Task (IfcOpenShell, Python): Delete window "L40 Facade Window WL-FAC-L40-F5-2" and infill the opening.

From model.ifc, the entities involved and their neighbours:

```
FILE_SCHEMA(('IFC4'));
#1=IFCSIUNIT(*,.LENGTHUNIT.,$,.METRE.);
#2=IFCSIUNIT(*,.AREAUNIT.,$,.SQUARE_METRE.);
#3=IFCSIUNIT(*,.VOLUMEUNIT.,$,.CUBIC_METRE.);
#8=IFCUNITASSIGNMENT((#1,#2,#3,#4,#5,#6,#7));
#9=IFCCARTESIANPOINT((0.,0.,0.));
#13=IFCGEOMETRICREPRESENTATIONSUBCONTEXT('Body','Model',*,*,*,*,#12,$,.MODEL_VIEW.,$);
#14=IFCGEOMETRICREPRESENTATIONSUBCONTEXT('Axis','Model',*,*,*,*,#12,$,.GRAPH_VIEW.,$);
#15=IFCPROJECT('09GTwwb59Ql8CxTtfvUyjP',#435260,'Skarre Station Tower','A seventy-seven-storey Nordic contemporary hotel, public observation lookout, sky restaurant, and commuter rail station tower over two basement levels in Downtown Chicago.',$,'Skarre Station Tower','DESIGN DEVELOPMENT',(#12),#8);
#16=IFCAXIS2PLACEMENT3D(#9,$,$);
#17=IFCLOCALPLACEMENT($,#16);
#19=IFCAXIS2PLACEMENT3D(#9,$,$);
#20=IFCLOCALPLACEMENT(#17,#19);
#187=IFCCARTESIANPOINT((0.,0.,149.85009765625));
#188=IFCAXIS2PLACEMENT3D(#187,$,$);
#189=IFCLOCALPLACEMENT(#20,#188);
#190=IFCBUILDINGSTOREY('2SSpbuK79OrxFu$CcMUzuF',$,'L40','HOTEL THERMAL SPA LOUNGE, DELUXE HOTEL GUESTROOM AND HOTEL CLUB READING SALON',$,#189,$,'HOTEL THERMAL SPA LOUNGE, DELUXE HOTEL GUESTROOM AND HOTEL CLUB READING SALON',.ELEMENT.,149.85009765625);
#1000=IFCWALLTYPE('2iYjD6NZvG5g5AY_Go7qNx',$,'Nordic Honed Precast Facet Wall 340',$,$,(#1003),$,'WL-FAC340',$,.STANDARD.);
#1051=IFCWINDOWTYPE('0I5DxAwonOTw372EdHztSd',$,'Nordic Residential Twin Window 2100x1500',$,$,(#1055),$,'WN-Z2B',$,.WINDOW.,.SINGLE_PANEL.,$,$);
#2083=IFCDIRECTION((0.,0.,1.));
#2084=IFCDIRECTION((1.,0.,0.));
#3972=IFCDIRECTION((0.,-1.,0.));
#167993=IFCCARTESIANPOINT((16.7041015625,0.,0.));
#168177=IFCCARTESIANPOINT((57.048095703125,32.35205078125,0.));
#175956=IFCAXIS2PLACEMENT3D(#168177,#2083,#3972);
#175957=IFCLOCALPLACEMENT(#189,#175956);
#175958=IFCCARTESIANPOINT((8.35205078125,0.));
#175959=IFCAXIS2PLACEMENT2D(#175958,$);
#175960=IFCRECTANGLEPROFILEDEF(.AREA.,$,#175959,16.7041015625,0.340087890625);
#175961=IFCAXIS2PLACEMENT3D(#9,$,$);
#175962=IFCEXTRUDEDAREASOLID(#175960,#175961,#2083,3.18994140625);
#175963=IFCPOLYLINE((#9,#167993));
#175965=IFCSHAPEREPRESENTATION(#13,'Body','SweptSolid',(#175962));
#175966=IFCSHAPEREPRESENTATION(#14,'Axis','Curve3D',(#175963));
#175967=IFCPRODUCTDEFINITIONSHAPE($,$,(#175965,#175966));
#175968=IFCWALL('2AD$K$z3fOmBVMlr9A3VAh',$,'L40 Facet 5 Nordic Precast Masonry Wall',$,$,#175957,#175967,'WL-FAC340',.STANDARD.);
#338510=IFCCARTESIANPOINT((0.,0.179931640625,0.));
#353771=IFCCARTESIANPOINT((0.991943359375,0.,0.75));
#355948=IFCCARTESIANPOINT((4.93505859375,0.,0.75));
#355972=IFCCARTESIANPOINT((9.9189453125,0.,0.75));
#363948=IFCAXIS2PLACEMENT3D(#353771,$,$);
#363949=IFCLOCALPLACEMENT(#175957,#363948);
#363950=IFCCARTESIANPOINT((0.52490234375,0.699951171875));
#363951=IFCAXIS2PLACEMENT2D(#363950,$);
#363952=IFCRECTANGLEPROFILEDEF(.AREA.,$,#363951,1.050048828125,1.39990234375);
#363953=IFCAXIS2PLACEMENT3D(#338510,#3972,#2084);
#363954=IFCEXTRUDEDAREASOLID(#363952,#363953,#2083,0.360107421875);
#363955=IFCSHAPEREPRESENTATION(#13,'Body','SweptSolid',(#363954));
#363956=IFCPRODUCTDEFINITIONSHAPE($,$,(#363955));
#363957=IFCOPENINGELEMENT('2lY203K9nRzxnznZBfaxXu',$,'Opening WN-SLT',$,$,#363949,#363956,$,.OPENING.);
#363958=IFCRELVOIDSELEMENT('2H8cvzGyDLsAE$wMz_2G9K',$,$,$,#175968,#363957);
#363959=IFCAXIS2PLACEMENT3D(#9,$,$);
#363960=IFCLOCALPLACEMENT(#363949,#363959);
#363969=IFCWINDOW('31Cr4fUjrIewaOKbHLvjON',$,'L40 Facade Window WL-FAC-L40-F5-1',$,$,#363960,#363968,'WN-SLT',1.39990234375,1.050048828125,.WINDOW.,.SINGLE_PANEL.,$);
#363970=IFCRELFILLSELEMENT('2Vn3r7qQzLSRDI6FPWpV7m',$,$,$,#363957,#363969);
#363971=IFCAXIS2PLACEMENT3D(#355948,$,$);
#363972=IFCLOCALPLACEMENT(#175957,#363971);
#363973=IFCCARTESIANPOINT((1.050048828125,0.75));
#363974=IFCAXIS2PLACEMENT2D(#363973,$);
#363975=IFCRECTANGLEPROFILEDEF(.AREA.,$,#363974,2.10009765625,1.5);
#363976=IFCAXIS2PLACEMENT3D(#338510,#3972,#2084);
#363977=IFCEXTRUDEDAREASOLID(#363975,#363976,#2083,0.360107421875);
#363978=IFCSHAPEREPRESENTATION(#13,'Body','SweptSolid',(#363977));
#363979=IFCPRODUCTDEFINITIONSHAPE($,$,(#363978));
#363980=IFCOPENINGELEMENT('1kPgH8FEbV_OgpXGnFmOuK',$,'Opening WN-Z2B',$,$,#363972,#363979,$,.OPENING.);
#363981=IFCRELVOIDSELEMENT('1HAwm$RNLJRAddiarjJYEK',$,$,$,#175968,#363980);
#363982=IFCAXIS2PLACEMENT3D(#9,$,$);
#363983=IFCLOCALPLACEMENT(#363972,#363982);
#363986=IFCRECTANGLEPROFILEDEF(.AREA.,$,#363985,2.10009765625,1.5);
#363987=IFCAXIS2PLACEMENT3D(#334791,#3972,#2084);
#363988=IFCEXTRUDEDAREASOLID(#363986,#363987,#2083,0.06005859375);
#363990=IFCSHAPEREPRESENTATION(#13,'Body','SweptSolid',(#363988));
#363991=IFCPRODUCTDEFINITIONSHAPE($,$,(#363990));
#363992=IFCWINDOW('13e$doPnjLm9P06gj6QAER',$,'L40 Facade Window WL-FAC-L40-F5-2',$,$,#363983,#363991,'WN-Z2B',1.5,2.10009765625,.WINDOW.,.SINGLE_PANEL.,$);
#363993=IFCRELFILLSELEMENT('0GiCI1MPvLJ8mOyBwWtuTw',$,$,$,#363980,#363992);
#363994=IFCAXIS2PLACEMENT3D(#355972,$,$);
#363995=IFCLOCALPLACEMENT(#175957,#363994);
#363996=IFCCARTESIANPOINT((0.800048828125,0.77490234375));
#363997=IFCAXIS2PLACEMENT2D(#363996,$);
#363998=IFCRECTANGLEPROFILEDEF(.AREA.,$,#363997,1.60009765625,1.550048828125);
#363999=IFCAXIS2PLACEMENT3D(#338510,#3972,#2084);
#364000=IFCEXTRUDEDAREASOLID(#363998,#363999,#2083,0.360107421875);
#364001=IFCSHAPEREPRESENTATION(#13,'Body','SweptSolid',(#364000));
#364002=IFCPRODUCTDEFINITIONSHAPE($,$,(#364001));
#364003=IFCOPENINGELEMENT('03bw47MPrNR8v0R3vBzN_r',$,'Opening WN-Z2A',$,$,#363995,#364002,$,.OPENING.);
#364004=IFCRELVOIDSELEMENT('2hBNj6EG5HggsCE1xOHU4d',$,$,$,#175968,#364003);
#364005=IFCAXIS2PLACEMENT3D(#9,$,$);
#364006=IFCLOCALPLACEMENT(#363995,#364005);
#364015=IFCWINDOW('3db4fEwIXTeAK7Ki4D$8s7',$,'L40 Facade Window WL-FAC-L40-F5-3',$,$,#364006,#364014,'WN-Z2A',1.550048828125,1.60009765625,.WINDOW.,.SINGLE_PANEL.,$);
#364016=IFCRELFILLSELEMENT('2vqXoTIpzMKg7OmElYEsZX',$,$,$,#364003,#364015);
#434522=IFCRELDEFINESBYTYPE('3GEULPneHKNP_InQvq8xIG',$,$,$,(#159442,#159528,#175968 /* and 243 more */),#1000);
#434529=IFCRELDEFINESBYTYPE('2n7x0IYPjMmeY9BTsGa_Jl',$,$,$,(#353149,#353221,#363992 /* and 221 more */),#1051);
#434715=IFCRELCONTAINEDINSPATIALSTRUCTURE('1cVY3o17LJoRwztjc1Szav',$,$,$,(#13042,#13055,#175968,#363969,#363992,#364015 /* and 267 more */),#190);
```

```python
import ifcopenshell
import ifcopenshell.api.feature
import ifcopenshell.api.root
import ifcopenshell.geom
import ifcopenshell.util.shape

model = ifcopenshell.open("model.ifc")
settings = ifcopenshell.geom.settings()


def volume(element):
    """Net volume in cubic metres, openings subtracted."""
    shape = ifcopenshell.geom.create_shape(settings, element)
    return ifcopenshell.util.shape.get_volume(shape.geometry)


window = model.by_id(363992)
opening = window.FillsVoids[0].RelatingOpeningElement
wall = opening.VoidsElements[0].RelatingBuildingElement
before = volume(wall)

ifcopenshell.api.root.remove_product(model, product=window)
ifcopenshell.api.feature.remove_feature(model, feature=opening)

after = volume(wall)

print(f"wall volume {before:.3f} -> {after:.3f} m3")

model.write("model_updated.ifc")
```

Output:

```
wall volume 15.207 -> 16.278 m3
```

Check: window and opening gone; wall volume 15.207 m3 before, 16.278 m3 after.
